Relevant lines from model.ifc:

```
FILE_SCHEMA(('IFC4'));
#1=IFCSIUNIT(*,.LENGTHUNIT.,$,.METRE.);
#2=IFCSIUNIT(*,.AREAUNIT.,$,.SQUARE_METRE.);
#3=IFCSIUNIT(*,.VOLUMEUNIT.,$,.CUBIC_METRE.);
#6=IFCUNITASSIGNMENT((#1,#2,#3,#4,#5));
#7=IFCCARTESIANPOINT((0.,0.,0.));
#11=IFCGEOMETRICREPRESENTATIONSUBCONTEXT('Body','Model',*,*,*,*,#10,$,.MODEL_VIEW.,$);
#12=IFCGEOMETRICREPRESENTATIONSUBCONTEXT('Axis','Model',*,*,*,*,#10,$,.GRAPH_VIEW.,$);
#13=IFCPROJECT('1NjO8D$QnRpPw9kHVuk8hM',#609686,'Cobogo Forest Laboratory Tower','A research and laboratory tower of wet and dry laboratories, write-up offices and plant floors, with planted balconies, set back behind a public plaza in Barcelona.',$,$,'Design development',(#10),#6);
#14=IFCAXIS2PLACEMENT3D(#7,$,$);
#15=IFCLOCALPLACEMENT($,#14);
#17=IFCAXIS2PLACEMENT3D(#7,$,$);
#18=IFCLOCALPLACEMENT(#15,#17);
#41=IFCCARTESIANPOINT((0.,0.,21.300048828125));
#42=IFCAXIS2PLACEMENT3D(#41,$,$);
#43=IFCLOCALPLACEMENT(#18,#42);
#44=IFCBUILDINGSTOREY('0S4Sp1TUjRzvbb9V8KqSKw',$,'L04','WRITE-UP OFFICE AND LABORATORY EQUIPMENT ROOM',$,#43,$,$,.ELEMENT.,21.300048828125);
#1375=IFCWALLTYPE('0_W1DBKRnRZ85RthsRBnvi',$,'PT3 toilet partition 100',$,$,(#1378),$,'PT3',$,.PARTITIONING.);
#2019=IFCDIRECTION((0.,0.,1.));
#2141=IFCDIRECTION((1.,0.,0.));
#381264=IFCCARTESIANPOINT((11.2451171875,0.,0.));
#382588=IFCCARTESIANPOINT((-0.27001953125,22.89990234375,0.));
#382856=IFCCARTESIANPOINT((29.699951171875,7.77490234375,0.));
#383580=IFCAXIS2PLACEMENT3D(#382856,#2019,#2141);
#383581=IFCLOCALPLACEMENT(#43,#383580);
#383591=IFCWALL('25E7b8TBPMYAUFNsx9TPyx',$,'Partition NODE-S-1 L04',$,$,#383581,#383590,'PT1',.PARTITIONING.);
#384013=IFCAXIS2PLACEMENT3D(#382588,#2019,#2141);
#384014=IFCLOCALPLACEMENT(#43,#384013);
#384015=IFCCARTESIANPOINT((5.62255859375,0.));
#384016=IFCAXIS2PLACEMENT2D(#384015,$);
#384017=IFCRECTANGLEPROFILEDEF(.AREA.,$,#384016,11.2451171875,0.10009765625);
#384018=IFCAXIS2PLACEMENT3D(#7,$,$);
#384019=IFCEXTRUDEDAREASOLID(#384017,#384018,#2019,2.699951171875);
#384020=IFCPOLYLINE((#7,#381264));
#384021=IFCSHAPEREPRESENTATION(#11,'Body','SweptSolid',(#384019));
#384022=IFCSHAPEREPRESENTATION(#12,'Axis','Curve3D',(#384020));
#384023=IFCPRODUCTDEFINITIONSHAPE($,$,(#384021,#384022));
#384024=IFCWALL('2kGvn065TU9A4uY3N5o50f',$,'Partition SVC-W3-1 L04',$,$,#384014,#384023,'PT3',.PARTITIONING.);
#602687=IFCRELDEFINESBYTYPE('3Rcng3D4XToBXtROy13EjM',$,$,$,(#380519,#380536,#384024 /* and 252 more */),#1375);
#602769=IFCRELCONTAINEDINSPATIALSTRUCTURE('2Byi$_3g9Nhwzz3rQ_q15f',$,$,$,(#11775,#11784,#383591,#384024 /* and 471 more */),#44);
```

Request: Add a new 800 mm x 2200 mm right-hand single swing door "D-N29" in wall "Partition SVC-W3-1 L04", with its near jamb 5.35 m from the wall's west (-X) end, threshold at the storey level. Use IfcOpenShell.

```python
import numpy as np
import ifcopenshell
import ifcopenshell.api.feature
import ifcopenshell.api.geometry
import ifcopenshell.api.root
import ifcopenshell.api.spatial
import ifcopenshell.geom
import ifcopenshell.util.element
import ifcopenshell.util.placement
import ifcopenshell.util.representation
import ifcopenshell.util.shape
import ifcopenshell.util.unit

model = ifcopenshell.open("model.ifc")
unit_scale = ifcopenshell.util.unit.calculate_unit_scale(model)
settings = ifcopenshell.geom.settings()


def volume(element):
    """Net volume in cubic metres, openings subtracted."""
    shape = ifcopenshell.geom.create_shape(settings, element)
    return ifcopenshell.util.shape.get_volume(shape.geometry)


wall = model.by_guid("2kGvn065TU9A4uY3N5o50f")
storey = ifcopenshell.util.element.get_container(wall, ifc_class="IfcBuildingStorey")
context = ifcopenshell.util.representation.get_context(model, "Model", "Body", "MODEL_VIEW")
before = volume(wall)

width, height, from_end, sill = 0.8, 2.2, 5.35, 0.0  # metres

# The wall runs along its own X axis, and the end named is its -X end.
wall_shape = ifcopenshell.geom.create_shape(settings, wall)
x, y, z = ifcopenshell.util.shape.get_vertices(wall_shape.geometry).T
start = x.min() + from_end
face, thickness = float(y.min()), float(y.max() - y.min())
wall_matrix = ifcopenshell.util.placement.get_local_placement(wall.ObjectPlacement)
level = ifcopenshell.util.placement.get_local_placement(storey.ObjectPlacement)[2, 3]


def in_wall(x, y):
    """Placement at x, y metres in the wall's axes, at sill height."""
    matrix = wall_matrix.copy()
    matrix[:, 3] = wall_matrix @ np.array([x / unit_scale, y / unit_scale, 0.0, 1.0])
    matrix[2, 3] = level + sill / unit_scale
    return matrix


# Opening: a box that overshoots both wall faces by 50 mm.
opening = ifcopenshell.api.root.create_entity(model, ifc_class="IfcOpeningElement", predefined_type="OPENING")
box = ifcopenshell.api.geometry.add_wall_representation(
    model, context=context, length=width, height=height, thickness=thickness + 0.1
)
ifcopenshell.api.geometry.assign_representation(model, product=opening, representation=box)
ifcopenshell.api.geometry.edit_object_placement(model, product=opening, matrix=in_wall(start, face - 0.05), is_si=False)
ifcopenshell.api.feature.add_feature(model, feature=opening, element=wall)

door = ifcopenshell.api.root.create_entity(model, ifc_class="IfcDoor", name="D-N29", predefined_type="DOOR")
door.OverallWidth, door.OverallHeight = width / unit_scale, height / unit_scale
door.OperationType = "SINGLE_SWING_RIGHT"
body = ifcopenshell.api.geometry.add_door_representation(
    model,
    context=context,
    overall_width=door.OverallWidth,
    overall_height=door.OverallHeight,
    operation_type="SINGLE_SWING_RIGHT",
    lining_properties={"LiningDepth": thickness / unit_scale, "ThresholdDepth": thickness / unit_scale},
)
ifcopenshell.api.geometry.assign_representation(model, product=door, representation=body)
ifcopenshell.api.spatial.assign_container(model, products=[door], relating_structure=storey)
ifcopenshell.api.feature.add_filling(model, opening=opening, element=door)

# The lining spans the wall, so the door starts at the wall face.
ifcopenshell.api.geometry.edit_object_placement(model, product=door, matrix=in_wall(start, face), is_si=False)

after = volume(wall)

print(f"wall volume {before:.3f} -> {after:.3f} m3")

model.write("model_rev.ifc")
```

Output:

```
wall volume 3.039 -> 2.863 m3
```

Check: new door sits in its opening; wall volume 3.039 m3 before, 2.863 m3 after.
